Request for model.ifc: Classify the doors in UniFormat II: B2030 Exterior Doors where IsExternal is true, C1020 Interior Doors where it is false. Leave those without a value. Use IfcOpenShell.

First a look at what the model holds.

```python
import ifcopenshell
import ifcopenshell.util.element

model = ifcopenshell.open("model.ifc")
print(model.schema)
print("classifications:", [c.Name for c in model.by_type("IfcClassification")])
values = [ifcopenshell.util.element.get_pset(e, "Pset_DoorCommon", "IsExternal") for e in model.by_type("IfcDoor")]
for value in (True, False, None):
    print("IsExternal", value, values.count(value))
```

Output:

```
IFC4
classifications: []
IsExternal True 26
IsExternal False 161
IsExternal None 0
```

```python
import ifcopenshell
import ifcopenshell.api.classification
import ifcopenshell.util.element

model = ifcopenshell.open("model.ifc")

system = ifcopenshell.api.classification.add_classification(model, classification="UniFormat II")

doors = model.by_type("IfcDoor")
external = {e: ifcopenshell.util.element.get_pset(e, "Pset_DoorCommon", "IsExternal") for e in doors}
for flag, code, name in ((True, "B2030", "Exterior Doors"), (False, "C1020", "Interior Doors")):
    products = [e for e in doors if external[e] is flag]
    ifcopenshell.api.classification.add_reference(
        model, products=products, classification=system, identification=code, name=name
    )
    print(code, len(products))

model.write("model_rev.ifc")
```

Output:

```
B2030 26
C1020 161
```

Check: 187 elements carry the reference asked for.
